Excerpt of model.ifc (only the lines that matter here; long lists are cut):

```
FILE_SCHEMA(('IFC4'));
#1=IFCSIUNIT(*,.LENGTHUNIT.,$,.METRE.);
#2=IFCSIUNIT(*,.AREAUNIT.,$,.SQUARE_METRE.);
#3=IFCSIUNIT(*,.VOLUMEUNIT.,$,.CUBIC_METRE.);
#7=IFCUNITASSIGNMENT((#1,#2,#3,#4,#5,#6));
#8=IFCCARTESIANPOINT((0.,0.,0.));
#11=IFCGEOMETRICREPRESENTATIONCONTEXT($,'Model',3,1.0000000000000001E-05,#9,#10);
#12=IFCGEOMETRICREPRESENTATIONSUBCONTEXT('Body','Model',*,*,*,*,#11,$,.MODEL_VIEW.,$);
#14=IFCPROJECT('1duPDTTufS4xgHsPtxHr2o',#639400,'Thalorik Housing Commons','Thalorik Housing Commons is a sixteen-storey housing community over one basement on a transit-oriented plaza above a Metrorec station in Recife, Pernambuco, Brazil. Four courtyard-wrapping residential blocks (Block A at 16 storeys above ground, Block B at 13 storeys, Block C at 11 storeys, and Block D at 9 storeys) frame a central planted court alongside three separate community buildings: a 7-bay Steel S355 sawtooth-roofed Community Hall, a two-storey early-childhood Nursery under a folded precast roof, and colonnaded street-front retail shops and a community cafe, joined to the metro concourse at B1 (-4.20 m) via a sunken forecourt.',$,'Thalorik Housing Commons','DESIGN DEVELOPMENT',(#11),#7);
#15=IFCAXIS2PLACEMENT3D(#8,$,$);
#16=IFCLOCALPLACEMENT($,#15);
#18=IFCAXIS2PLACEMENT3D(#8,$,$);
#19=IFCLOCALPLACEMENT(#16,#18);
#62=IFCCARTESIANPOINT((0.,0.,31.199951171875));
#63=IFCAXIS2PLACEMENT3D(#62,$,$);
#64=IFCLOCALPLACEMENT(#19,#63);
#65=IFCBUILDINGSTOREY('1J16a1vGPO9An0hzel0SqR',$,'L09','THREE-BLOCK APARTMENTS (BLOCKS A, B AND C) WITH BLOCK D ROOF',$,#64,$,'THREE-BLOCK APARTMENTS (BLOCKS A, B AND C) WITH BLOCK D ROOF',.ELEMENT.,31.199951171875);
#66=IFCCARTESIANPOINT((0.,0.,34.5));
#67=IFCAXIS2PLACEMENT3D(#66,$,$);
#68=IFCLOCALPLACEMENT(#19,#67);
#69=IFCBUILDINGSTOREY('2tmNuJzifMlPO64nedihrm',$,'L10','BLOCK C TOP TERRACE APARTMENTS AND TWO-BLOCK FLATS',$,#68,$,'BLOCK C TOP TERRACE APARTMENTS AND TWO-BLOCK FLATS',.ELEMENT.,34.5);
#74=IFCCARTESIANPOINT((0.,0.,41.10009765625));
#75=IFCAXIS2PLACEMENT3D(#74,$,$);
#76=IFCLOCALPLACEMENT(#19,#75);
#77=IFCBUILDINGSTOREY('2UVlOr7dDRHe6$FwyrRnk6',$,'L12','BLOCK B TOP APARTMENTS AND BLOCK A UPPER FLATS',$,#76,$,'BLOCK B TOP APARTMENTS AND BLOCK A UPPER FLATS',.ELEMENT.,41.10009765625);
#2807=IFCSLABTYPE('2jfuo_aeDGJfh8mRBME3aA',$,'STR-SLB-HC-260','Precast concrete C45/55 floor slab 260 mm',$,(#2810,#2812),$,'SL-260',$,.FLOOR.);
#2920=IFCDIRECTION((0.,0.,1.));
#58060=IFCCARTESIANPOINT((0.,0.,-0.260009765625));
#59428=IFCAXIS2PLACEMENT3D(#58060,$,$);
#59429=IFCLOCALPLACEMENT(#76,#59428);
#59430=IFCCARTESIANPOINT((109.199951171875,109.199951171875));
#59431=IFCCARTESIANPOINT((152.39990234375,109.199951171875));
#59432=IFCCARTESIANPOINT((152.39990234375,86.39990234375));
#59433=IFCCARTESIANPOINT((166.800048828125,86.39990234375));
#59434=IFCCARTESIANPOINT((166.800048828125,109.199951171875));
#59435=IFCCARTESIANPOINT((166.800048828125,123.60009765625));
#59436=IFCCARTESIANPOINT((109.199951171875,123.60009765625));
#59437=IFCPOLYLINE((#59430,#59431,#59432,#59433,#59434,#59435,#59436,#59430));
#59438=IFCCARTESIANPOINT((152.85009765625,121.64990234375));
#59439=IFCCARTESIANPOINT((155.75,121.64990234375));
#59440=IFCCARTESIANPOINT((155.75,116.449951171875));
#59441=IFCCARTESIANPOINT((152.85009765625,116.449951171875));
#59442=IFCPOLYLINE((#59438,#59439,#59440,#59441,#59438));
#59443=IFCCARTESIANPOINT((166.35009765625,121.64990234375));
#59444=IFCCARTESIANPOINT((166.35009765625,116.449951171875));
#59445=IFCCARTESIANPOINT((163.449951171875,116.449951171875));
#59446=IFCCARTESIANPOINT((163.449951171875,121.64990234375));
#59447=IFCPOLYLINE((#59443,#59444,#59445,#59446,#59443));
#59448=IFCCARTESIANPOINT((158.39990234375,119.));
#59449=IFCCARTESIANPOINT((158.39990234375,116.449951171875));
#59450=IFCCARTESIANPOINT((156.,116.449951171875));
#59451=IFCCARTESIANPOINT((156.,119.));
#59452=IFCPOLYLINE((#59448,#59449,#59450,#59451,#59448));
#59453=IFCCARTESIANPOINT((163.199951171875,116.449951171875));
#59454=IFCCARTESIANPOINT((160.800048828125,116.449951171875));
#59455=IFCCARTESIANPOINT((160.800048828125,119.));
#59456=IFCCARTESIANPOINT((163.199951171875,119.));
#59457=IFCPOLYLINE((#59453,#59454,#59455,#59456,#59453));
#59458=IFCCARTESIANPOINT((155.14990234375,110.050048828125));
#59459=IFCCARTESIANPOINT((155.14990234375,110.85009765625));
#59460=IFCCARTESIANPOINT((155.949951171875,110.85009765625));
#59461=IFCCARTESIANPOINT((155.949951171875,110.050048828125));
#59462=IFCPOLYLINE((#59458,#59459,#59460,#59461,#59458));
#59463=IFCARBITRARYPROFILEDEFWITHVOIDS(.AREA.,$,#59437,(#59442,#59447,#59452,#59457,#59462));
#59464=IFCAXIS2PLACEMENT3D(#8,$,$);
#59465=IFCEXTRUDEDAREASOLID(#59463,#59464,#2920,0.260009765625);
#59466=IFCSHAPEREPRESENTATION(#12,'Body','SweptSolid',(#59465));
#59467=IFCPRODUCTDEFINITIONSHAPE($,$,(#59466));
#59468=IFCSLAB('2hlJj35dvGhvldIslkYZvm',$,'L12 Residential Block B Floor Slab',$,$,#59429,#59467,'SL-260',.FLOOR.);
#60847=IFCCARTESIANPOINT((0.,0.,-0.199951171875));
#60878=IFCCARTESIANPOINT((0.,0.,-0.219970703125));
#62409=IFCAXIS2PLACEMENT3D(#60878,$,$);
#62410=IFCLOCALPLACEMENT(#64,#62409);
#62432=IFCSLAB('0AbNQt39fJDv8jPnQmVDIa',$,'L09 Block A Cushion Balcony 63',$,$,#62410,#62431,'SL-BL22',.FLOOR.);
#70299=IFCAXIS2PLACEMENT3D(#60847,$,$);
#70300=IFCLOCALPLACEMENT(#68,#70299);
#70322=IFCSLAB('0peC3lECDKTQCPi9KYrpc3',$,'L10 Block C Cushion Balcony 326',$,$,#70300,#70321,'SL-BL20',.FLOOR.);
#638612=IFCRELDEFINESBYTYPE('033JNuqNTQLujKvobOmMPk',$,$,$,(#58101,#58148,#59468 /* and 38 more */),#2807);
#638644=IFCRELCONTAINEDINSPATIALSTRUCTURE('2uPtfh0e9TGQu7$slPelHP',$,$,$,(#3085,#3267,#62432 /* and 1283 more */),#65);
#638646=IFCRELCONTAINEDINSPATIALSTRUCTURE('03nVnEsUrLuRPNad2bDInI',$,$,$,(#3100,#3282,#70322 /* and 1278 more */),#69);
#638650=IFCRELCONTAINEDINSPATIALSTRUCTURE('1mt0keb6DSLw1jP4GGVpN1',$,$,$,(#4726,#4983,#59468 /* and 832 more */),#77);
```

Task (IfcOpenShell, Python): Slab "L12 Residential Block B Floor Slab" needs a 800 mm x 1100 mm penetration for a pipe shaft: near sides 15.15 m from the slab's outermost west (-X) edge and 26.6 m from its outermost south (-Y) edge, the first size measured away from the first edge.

```python
import numpy as np
import ifcopenshell
import ifcopenshell.api.feature
import ifcopenshell.api.geometry
import ifcopenshell.api.root
import ifcopenshell.geom
import ifcopenshell.util.placement
import ifcopenshell.util.representation
import ifcopenshell.util.shape
import ifcopenshell.util.unit

model = ifcopenshell.open("model.ifc")
unit_scale = ifcopenshell.util.unit.calculate_unit_scale(model)
settings = ifcopenshell.geom.settings()


def volume(element):
    """Net volume in cubic metres, openings subtracted."""
    shape = ifcopenshell.geom.create_shape(settings, element)
    return ifcopenshell.util.shape.get_volume(shape.geometry)


slab = model.by_guid("2hlJj35dvGhvldIslkYZvm")
before = volume(slab)

# Extent in the slab's own axes, in metres. The edges named are its -X and -Y sides.
slab_shape = ifcopenshell.geom.create_shape(settings, slab)
vertices = ifcopenshell.util.shape.get_vertices(slab_shape.geometry)
x_min, y_min, bottom = vertices.min(axis=0)
top = vertices[:, 2].max()

opening = ifcopenshell.api.root.create_entity(model, ifc_class="IfcOpeningElement", name="Pipe shaft opening", predefined_type="OPENING")
context = ifcopenshell.util.representation.get_context(model, "Model", "Body", "MODEL_VIEW")
width, depth = 0.8, 1.1
outline = [(0.0, 0.0), (width, 0.0), (width, depth), (0.0, depth), (0.0, 0.0)]
# Overshoot both faces by 50 mm so the cut is clean.
shape = ifcopenshell.api.geometry.add_slab_representation(
    model, context=context, depth=top - bottom + 0.1, polyline=outline
)
ifcopenshell.api.geometry.assign_representation(model, product=opening, representation=shape)

matrix = ifcopenshell.util.placement.get_local_placement(slab.ObjectPlacement)
matrix[:, 3] = matrix @ np.append(np.array([x_min + 15.15, y_min + 26.6, bottom - 0.05]) / unit_scale, 1.0)
ifcopenshell.api.geometry.edit_object_placement(model, product=opening, matrix=matrix, is_si=False)
ifcopenshell.api.feature.add_feature(model, feature=opening, element=slab)

after = volume(slab)

print(f"slab volume {before:.3f} -> {after:.3f} m3")

model.write("model-out.ifc")
```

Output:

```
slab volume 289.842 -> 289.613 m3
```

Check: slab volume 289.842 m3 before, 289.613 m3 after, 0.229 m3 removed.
